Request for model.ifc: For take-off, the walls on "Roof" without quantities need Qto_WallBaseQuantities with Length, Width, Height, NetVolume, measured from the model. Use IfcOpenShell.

First a look at what the model holds.

```python
import ifcopenshell
import ifcopenshell.util.element
import ifcopenshell.util.unit

model = ifcopenshell.open("model.ifc")
print(model.schema)
for unit_type in ("LENGTHUNIT", "AREAUNIT", "VOLUMEUNIT"):
    print(unit_type, ifcopenshell.util.unit.calculate_unit_scale(model, unit_type))
storey = next(s for s in model.by_type("IfcBuildingStorey") if s.Name == "Roof")
walls = [e for e in ifcopenshell.util.element.get_decomposition(storey) if e.is_a("IfcWall")]
for e in sorted(walls, key=lambda e: e.id()):
    print(e.id(), e.is_a(), e.Name, list(ifcopenshell.util.element.get_psets(e, qtos_only=True)), sep=" | ")
```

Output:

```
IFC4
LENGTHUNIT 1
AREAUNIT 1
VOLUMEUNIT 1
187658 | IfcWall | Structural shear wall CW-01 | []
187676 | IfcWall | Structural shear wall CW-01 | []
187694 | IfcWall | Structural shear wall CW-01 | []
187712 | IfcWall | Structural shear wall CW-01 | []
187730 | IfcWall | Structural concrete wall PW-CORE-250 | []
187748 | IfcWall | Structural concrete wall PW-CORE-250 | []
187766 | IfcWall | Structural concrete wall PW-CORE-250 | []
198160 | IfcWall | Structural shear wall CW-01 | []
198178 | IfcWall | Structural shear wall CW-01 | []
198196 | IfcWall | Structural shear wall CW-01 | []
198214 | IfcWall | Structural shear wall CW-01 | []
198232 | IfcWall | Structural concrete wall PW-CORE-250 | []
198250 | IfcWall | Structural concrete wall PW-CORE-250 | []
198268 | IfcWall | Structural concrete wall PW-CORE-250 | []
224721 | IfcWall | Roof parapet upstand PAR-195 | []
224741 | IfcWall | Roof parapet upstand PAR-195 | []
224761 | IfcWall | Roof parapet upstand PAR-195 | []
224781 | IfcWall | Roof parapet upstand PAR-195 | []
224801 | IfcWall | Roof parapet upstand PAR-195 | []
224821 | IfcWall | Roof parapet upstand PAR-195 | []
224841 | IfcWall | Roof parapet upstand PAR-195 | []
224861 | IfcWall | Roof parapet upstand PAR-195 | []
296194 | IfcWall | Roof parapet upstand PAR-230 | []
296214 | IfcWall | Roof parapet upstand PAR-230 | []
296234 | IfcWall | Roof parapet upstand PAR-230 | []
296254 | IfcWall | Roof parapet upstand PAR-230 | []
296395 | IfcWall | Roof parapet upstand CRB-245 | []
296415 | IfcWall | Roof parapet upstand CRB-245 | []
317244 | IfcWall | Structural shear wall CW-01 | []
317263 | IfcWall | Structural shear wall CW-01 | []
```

```python
import ifcopenshell
import ifcopenshell.api.pset
import ifcopenshell.geom
import ifcopenshell.util.element
import ifcopenshell.util.shape
import ifcopenshell.util.unit

model = ifcopenshell.open("model.ifc")
unit_scale = ifcopenshell.util.unit.calculate_unit_scale(model)
volume_scale = ifcopenshell.util.unit.calculate_unit_scale(model, "VOLUMEUNIT")
settings = ifcopenshell.geom.settings()

storey = next(s for s in model.by_type("IfcBuildingStorey") if s.Name == "Roof")
walls = [e for e in ifcopenshell.util.element.get_decomposition(storey) if e.is_a("IfcWall")]

for e in sorted(walls, key=lambda e: e.id()):
    if ifcopenshell.util.element.get_psets(e, qtos_only=True, should_inherit=False):
        continue
    # Geometry comes back in metres, in the element's own axes.
    shape = ifcopenshell.geom.create_shape(settings, e)
    values = {
        "Length": ifcopenshell.util.shape.get_x(shape.geometry) / unit_scale,
        "Width": ifcopenshell.util.shape.get_y(shape.geometry) / unit_scale,
        "Height": ifcopenshell.util.shape.get_z(shape.geometry) / unit_scale,
        "NetVolume": ifcopenshell.util.shape.get_volume(shape.geometry) / volume_scale,
    }
    qto = ifcopenshell.api.pset.add_qto(model, product=e, name="Qto_WallBaseQuantities")
    ifcopenshell.api.pset.edit_qto(model, qto=qto, properties=values)
    print(e.id(), {k: round(v, 3) for k, v in values.items()})

model.write("model_v2.ifc")
```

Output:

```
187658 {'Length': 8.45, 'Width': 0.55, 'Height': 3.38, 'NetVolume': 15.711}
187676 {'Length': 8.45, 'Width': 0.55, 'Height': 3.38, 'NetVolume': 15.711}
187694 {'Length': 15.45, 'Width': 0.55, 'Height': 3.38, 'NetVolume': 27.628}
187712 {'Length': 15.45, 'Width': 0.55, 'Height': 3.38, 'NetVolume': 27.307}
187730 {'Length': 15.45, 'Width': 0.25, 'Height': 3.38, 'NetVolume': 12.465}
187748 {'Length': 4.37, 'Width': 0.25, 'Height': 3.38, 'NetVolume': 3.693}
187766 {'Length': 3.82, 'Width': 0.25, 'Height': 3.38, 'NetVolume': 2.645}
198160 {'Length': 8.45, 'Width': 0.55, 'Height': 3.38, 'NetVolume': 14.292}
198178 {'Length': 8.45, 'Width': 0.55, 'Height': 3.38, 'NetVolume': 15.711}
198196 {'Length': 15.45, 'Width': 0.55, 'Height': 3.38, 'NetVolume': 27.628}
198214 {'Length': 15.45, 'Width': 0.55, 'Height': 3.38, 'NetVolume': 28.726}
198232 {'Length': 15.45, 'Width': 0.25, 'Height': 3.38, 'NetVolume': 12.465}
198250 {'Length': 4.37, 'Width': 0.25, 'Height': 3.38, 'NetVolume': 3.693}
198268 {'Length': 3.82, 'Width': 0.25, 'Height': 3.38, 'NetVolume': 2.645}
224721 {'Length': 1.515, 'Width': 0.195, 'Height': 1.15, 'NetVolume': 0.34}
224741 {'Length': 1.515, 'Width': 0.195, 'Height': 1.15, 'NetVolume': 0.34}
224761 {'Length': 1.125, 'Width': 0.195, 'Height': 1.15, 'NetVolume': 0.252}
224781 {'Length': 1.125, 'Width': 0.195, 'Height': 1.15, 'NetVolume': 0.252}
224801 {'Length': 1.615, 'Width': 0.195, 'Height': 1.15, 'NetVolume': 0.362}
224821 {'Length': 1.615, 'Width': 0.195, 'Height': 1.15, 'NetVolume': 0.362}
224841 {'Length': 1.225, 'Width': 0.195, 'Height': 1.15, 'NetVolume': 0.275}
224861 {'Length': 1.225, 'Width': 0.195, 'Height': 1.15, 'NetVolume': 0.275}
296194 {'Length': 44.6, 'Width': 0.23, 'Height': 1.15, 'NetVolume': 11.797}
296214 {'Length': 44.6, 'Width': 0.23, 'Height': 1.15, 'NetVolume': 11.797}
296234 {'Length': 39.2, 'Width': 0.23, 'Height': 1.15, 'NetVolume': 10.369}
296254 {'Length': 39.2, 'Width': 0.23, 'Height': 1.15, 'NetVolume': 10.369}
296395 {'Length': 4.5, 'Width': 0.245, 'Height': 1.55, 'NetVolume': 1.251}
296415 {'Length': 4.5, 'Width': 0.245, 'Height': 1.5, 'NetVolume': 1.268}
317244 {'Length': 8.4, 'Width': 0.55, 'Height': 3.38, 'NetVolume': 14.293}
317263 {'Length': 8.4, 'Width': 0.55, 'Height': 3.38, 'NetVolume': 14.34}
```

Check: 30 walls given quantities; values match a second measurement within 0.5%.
